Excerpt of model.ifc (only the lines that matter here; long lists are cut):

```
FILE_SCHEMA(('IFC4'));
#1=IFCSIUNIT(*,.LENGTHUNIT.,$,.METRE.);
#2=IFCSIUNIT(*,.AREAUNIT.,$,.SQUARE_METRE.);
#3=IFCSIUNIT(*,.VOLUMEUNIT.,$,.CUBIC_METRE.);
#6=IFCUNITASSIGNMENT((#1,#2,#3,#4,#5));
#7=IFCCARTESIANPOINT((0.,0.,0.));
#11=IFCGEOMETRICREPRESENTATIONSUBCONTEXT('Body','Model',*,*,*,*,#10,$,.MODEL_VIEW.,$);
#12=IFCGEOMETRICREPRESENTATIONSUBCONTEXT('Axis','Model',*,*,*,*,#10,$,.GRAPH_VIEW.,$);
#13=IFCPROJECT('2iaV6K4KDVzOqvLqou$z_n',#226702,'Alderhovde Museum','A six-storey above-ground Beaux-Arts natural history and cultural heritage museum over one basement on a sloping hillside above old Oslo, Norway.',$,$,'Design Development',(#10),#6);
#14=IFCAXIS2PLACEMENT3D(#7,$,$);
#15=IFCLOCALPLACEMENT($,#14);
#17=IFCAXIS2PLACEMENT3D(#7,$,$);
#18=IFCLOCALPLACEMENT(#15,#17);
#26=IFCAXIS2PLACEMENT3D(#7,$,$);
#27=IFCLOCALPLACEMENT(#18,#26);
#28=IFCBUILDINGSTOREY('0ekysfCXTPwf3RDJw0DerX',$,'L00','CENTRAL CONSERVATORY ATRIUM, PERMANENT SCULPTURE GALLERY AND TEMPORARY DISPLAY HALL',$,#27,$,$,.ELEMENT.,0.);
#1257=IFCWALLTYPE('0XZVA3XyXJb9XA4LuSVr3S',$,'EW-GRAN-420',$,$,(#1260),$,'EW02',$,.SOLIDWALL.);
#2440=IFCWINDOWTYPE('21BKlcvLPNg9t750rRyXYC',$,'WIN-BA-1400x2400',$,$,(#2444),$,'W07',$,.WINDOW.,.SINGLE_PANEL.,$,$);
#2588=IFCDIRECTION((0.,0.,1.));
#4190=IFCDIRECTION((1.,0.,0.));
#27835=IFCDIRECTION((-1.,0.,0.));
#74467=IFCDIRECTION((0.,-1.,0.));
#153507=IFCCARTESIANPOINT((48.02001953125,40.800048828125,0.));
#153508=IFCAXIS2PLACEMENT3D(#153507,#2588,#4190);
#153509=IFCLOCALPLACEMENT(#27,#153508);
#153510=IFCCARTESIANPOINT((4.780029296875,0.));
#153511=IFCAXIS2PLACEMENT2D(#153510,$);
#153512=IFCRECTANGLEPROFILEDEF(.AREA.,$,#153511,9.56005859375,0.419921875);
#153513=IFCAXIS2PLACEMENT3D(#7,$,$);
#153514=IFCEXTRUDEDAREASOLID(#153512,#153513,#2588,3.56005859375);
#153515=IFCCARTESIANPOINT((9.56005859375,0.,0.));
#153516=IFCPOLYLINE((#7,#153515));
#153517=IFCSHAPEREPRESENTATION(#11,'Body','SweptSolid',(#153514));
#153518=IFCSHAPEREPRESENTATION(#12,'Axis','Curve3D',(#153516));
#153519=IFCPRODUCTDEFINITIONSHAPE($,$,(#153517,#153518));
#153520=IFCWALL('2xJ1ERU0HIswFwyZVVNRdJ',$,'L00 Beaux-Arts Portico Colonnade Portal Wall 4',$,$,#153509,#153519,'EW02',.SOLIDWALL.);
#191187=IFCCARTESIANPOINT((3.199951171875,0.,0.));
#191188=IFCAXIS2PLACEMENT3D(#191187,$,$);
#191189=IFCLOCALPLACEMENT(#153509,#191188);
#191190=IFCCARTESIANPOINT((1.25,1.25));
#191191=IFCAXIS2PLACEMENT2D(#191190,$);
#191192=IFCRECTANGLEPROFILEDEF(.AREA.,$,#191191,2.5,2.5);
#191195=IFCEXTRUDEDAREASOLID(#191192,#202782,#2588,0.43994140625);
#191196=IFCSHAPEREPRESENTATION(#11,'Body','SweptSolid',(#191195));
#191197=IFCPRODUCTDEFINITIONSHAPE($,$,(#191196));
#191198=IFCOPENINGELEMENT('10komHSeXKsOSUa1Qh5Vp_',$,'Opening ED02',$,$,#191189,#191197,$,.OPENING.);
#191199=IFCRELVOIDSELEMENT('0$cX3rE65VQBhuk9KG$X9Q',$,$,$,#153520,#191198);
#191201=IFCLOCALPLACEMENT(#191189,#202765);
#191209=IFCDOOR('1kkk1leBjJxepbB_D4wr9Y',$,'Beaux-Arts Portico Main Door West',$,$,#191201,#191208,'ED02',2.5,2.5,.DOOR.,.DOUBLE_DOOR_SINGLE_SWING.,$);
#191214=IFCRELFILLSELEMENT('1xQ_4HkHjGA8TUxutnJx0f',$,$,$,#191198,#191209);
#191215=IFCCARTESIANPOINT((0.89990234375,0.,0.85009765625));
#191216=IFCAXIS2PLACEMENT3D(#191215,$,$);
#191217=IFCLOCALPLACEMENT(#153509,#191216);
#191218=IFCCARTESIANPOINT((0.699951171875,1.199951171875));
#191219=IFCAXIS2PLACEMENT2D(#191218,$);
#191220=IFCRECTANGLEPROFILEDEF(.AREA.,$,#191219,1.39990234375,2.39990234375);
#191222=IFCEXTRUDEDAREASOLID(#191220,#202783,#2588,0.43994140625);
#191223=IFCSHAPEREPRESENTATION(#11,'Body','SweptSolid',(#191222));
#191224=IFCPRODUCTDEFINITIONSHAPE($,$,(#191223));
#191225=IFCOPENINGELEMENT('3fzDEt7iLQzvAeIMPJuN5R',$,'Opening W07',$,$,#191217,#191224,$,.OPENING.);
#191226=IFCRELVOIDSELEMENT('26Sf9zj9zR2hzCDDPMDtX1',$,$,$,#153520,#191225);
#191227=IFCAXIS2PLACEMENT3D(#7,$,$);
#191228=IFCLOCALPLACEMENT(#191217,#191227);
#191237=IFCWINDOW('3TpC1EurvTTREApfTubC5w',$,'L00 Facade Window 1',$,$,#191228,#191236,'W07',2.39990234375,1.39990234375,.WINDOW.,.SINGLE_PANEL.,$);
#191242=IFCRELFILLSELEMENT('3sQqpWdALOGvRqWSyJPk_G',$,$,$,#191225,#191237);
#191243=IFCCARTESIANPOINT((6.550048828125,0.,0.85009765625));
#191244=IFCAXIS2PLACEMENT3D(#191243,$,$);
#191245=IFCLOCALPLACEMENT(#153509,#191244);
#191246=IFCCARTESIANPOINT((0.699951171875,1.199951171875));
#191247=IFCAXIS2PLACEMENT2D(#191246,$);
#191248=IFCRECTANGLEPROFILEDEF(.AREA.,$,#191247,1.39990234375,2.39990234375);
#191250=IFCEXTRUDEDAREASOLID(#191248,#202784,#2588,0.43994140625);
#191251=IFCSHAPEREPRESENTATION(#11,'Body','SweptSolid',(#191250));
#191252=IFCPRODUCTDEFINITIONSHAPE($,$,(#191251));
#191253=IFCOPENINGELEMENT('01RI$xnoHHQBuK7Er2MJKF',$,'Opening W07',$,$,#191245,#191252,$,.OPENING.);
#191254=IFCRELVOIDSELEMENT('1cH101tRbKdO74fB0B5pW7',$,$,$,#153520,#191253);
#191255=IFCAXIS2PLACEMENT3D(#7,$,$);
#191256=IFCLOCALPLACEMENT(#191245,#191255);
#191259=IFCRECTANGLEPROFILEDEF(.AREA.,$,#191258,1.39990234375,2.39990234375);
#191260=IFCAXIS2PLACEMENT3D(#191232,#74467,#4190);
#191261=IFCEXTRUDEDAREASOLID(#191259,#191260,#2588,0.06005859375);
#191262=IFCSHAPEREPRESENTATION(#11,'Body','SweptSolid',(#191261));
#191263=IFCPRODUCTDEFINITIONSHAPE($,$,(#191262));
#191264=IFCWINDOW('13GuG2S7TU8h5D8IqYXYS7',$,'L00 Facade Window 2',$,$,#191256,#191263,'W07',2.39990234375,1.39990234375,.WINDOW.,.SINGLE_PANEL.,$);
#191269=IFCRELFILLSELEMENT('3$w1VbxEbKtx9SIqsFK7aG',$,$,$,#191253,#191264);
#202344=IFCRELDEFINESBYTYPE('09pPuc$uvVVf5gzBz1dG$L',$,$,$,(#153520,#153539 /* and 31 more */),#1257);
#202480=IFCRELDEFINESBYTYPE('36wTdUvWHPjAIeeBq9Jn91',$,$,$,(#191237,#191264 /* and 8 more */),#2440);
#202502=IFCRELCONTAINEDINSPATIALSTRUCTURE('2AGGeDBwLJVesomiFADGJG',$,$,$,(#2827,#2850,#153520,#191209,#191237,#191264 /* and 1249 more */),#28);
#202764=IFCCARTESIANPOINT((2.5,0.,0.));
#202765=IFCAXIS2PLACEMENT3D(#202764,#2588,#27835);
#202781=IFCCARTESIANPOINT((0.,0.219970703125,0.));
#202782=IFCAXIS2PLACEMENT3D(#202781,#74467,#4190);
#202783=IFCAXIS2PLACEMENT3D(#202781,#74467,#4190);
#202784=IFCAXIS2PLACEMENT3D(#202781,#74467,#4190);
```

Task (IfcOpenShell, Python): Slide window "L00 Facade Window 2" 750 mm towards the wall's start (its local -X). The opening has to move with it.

```python
import ifcopenshell
import ifcopenshell.api.geometry
import ifcopenshell.util.placement

model = ifcopenshell.open("model.ifc")

window = model.by_id(191264)
opening = window.FillsVoids[0].RelatingOpeningElement
wall = opening.VoidsElements[0].RelatingBuildingElement

wall_matrix = ifcopenshell.util.placement.get_local_placement(wall.ObjectPlacement)
shift = wall_matrix[:3, 0] * -0.75
before = ifcopenshell.util.placement.get_local_placement(window.ObjectPlacement)[:3, 3].copy()

# The window is placed relative to its opening, so it follows when the opening moves.
matrix = ifcopenshell.util.placement.get_local_placement(opening.ObjectPlacement)
matrix[:3, 3] += shift
ifcopenshell.api.geometry.edit_object_placement(
    model, product=opening, matrix=matrix, is_si=False, should_transform_children=True
)

after = ifcopenshell.util.placement.get_local_placement(window.ObjectPlacement)[:3, 3]
print("window moved by", (after - before).round(3) + 0.0)

model.write("model_updated.ifc")
```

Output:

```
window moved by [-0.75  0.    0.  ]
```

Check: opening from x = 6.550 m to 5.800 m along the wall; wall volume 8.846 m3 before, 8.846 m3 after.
